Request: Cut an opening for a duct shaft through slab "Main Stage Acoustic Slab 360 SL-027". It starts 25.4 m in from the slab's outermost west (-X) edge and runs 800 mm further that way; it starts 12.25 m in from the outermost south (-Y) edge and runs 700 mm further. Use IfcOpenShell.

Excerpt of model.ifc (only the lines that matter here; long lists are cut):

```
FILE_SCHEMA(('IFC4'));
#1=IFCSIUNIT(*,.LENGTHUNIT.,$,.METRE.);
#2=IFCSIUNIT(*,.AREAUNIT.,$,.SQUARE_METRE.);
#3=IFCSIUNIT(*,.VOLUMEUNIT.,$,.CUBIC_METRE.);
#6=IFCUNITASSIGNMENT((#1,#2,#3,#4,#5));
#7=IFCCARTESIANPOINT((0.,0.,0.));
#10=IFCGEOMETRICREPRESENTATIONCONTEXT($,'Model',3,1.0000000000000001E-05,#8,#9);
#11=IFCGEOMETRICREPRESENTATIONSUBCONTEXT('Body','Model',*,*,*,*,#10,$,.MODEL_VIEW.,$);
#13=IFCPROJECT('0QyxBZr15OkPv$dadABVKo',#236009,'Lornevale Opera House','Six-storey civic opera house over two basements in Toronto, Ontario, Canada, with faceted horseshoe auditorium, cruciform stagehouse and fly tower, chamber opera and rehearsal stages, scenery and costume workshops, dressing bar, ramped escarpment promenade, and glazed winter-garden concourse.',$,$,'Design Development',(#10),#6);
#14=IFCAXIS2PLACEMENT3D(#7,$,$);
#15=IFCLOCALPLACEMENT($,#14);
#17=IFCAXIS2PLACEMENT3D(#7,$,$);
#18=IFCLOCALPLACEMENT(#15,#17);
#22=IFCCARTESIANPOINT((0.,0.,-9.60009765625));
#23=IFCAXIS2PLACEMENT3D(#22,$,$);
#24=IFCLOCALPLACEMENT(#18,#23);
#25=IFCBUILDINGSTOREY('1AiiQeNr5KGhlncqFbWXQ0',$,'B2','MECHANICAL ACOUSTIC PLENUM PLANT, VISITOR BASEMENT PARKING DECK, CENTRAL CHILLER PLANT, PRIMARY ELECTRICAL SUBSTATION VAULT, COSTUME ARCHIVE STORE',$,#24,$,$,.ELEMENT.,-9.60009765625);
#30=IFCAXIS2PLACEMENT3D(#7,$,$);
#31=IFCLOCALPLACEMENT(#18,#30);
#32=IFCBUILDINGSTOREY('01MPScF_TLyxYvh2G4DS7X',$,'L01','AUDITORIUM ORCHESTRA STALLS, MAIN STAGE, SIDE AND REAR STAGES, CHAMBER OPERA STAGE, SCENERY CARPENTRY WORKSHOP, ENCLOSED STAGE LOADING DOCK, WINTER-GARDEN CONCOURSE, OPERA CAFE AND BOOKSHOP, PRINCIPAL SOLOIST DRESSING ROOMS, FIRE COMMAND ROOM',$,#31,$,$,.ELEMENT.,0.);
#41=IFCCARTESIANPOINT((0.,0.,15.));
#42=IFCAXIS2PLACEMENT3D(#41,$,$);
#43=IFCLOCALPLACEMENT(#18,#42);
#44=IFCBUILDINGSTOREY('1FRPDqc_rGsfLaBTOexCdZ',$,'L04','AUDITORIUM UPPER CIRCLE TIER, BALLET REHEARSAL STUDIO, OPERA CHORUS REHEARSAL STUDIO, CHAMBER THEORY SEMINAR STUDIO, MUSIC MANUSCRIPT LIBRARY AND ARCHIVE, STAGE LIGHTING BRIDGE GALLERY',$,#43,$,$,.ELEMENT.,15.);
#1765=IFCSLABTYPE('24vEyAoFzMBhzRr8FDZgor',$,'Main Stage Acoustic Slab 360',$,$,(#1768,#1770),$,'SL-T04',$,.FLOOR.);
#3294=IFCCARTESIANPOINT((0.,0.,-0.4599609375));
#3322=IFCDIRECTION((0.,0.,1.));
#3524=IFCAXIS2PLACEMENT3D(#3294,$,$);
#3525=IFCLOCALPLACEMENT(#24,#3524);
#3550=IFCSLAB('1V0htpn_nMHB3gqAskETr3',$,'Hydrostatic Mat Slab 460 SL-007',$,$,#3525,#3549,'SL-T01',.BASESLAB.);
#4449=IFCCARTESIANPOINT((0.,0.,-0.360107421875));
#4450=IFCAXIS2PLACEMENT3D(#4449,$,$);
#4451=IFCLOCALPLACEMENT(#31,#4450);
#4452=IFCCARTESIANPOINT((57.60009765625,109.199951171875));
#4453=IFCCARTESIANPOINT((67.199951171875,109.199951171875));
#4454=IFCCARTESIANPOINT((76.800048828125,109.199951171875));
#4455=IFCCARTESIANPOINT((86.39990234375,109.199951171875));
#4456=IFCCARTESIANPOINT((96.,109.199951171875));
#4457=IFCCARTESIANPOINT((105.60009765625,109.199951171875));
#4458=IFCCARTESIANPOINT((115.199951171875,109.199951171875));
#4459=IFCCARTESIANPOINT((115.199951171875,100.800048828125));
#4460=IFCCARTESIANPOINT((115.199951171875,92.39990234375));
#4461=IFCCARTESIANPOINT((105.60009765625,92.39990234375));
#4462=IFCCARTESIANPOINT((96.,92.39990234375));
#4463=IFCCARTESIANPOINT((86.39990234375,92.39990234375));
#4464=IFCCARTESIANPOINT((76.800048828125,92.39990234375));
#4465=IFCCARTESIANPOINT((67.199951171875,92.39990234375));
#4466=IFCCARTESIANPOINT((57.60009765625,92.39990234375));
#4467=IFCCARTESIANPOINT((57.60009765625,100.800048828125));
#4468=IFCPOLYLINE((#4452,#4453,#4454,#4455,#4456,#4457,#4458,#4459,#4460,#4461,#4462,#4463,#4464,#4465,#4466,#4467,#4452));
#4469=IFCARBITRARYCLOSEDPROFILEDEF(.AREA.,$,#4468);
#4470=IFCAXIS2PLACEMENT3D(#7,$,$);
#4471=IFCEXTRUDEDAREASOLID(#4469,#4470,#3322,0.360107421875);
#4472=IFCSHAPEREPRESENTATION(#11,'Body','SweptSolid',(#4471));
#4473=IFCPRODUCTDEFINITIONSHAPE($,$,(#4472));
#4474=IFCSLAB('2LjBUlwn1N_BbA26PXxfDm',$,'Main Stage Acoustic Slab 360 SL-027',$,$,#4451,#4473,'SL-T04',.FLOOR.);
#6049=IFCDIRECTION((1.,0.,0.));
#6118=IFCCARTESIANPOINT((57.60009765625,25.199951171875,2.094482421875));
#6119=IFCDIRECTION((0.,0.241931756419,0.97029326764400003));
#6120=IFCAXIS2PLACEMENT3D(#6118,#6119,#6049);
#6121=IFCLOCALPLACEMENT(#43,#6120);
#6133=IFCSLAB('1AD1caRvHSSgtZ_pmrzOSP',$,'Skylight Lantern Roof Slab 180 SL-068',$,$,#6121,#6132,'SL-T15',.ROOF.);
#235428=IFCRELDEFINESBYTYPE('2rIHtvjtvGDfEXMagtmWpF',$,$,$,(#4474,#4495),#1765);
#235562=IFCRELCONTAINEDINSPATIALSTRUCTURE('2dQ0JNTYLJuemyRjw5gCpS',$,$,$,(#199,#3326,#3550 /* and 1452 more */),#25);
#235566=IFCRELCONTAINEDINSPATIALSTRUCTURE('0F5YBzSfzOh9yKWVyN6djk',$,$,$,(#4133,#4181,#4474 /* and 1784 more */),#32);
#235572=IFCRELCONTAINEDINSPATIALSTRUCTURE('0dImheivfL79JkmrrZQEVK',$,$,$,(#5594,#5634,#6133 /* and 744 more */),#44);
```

```python
import numpy as np
import ifcopenshell
import ifcopenshell.api.feature
import ifcopenshell.api.geometry
import ifcopenshell.api.root
import ifcopenshell.geom
import ifcopenshell.util.placement
import ifcopenshell.util.representation
import ifcopenshell.util.shape
import ifcopenshell.util.unit

model = ifcopenshell.open("model.ifc")
unit_scale = ifcopenshell.util.unit.calculate_unit_scale(model)
settings = ifcopenshell.geom.settings()


def volume(element):
    """Net volume in cubic metres, openings subtracted."""
    shape = ifcopenshell.geom.create_shape(settings, element)
    return ifcopenshell.util.shape.get_volume(shape.geometry)


slab = model.by_guid("2LjBUlwn1N_BbA26PXxfDm")
before = volume(slab)

# Extent in the slab's own axes, in metres. The edges named are its -X and -Y sides.
slab_shape = ifcopenshell.geom.create_shape(settings, slab)
vertices = ifcopenshell.util.shape.get_vertices(slab_shape.geometry)
x_min, y_min, bottom = vertices.min(axis=0)
top = vertices[:, 2].max()

opening = ifcopenshell.api.root.create_entity(model, ifc_class="IfcOpeningElement", name="Duct shaft opening", predefined_type="OPENING")
context = ifcopenshell.util.representation.get_context(model, "Model", "Body", "MODEL_VIEW")
width, depth = 0.8, 0.7
outline = [(0.0, 0.0), (width, 0.0), (width, depth), (0.0, depth), (0.0, 0.0)]
# Overshoot both faces by 50 mm so the cut is clean.
shape = ifcopenshell.api.geometry.add_slab_representation(
    model, context=context, depth=top - bottom + 0.1, polyline=outline
)
ifcopenshell.api.geometry.assign_representation(model, product=opening, representation=shape)

matrix = ifcopenshell.util.placement.get_local_placement(slab.ObjectPlacement)
matrix[:, 3] = matrix @ np.append(np.array([x_min + 25.4, y_min + 12.25, bottom - 0.05]) / unit_scale, 1.0)
ifcopenshell.api.geometry.edit_object_placement(model, product=opening, matrix=matrix, is_si=False)
ifcopenshell.api.feature.add_feature(model, feature=opening, element=slab)

after = volume(slab)

print(f"slab volume {before:.3f} -> {after:.3f} m3")

model.write("model_updated.ifc")
```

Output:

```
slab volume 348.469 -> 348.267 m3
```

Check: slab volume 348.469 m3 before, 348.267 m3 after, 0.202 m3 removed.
